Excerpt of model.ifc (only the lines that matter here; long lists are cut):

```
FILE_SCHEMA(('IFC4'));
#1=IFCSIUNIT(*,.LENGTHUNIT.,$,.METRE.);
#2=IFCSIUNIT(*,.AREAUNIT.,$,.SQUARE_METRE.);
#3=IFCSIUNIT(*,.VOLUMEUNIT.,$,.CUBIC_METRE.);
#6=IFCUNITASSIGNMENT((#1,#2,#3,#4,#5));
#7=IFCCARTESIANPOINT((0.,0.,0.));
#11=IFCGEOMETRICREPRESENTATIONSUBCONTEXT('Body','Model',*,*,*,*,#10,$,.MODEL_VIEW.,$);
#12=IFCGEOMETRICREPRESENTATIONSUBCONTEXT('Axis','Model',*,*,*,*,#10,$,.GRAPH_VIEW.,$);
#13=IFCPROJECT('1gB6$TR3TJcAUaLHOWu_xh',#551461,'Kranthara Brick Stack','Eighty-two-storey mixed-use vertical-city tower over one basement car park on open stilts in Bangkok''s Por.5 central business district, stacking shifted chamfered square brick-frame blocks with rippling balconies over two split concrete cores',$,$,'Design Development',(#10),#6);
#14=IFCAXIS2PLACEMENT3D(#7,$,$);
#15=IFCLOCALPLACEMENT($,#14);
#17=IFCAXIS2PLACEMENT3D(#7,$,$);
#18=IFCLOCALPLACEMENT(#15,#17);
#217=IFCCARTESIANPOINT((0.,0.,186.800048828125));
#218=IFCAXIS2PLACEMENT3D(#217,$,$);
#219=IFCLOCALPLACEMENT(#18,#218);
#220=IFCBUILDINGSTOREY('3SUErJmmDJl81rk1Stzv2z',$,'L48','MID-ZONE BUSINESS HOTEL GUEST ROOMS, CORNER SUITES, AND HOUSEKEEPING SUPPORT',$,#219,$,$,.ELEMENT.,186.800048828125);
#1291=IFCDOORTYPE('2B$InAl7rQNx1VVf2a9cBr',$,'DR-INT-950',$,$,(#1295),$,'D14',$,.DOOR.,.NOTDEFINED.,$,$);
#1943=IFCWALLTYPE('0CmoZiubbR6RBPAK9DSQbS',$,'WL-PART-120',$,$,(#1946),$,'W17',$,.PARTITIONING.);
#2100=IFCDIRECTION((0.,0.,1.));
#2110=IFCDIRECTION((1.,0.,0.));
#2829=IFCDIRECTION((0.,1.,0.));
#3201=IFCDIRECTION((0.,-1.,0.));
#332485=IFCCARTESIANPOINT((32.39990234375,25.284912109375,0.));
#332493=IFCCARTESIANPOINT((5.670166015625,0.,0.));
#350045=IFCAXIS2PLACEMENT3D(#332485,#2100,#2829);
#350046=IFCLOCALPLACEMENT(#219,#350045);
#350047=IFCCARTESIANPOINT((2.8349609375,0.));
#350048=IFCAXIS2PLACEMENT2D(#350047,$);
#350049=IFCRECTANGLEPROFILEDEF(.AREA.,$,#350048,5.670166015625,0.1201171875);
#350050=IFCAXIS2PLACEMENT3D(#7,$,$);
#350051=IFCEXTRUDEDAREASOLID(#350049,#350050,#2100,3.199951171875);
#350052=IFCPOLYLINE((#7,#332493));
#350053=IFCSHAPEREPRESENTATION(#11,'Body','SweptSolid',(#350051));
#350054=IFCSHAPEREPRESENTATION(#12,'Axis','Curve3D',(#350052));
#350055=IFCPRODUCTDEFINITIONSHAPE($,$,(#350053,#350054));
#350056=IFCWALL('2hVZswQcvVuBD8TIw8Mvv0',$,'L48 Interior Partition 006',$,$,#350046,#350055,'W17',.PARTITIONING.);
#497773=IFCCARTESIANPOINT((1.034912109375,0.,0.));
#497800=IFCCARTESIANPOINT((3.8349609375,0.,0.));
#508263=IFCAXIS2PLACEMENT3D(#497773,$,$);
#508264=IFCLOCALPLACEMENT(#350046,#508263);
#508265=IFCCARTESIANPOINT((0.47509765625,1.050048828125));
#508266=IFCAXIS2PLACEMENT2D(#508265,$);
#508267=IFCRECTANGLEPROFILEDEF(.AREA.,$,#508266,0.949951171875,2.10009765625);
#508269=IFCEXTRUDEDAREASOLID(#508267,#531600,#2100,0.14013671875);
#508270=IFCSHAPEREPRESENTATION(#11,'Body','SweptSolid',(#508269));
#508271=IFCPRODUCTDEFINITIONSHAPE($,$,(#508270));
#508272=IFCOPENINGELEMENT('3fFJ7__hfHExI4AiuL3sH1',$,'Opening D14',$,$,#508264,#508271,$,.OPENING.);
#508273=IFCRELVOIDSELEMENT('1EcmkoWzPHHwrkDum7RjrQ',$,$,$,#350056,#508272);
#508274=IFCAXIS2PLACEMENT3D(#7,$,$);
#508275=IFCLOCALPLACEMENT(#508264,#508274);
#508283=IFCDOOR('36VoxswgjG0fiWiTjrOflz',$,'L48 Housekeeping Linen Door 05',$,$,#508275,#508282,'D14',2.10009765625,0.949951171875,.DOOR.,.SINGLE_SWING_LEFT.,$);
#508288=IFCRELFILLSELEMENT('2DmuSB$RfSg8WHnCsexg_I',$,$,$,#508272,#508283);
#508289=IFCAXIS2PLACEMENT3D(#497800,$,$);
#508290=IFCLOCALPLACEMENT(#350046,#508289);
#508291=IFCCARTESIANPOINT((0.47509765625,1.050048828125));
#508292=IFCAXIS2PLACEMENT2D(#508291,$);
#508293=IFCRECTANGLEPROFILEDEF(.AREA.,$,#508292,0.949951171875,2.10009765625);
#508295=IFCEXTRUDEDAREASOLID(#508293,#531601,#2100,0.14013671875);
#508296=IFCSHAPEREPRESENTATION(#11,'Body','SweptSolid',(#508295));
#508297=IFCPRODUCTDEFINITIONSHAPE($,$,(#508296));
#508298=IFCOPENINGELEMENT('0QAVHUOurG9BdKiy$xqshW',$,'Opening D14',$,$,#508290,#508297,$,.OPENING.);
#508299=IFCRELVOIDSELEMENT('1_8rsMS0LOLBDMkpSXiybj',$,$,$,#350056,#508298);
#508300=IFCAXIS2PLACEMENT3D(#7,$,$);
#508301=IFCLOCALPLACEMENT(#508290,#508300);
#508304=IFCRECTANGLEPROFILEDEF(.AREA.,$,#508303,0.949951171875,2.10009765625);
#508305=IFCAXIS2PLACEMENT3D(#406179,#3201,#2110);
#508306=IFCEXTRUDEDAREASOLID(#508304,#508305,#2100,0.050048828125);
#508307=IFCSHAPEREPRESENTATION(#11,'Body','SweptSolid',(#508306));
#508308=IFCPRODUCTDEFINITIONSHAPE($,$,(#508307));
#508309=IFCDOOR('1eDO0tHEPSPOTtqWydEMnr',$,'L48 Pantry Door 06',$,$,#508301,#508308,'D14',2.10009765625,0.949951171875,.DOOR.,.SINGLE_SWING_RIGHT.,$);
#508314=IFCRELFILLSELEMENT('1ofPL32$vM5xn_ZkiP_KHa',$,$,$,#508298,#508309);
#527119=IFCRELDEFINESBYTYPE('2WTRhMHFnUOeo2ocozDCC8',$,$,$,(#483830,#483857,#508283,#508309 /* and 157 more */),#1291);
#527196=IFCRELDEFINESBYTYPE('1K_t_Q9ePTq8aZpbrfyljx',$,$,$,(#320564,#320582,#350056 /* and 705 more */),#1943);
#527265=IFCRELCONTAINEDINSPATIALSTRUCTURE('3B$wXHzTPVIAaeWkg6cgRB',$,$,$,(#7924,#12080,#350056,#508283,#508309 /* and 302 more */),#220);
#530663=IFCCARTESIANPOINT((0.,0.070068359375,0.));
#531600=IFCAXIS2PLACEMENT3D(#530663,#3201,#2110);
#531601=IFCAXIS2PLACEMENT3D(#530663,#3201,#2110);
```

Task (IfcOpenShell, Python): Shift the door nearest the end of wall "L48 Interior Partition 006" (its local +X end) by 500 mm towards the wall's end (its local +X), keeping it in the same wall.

```python
import ifcopenshell
import ifcopenshell.api.geometry
import ifcopenshell.util.placement

model = ifcopenshell.open("model.ifc")

door = model.by_id(508309)
opening = door.FillsVoids[0].RelatingOpeningElement
wall = opening.VoidsElements[0].RelatingBuildingElement

wall_matrix = ifcopenshell.util.placement.get_local_placement(wall.ObjectPlacement)
shift = wall_matrix[:3, 0] * 0.5
before = ifcopenshell.util.placement.get_local_placement(door.ObjectPlacement)[:3, 3].copy()

# The door is placed relative to its opening, so it follows when the opening moves.
matrix = ifcopenshell.util.placement.get_local_placement(opening.ObjectPlacement)
matrix[:3, 3] += shift
ifcopenshell.api.geometry.edit_object_placement(
    model, product=opening, matrix=matrix, is_si=False, should_transform_children=True
)

after = ifcopenshell.util.placement.get_local_placement(door.ObjectPlacement)[:3, 3]
print("door moved by", (after - before).round(3) + 0.0)

model.write("model_rev.ifc")
```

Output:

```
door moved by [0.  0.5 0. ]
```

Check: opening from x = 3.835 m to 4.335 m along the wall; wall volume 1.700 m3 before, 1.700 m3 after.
